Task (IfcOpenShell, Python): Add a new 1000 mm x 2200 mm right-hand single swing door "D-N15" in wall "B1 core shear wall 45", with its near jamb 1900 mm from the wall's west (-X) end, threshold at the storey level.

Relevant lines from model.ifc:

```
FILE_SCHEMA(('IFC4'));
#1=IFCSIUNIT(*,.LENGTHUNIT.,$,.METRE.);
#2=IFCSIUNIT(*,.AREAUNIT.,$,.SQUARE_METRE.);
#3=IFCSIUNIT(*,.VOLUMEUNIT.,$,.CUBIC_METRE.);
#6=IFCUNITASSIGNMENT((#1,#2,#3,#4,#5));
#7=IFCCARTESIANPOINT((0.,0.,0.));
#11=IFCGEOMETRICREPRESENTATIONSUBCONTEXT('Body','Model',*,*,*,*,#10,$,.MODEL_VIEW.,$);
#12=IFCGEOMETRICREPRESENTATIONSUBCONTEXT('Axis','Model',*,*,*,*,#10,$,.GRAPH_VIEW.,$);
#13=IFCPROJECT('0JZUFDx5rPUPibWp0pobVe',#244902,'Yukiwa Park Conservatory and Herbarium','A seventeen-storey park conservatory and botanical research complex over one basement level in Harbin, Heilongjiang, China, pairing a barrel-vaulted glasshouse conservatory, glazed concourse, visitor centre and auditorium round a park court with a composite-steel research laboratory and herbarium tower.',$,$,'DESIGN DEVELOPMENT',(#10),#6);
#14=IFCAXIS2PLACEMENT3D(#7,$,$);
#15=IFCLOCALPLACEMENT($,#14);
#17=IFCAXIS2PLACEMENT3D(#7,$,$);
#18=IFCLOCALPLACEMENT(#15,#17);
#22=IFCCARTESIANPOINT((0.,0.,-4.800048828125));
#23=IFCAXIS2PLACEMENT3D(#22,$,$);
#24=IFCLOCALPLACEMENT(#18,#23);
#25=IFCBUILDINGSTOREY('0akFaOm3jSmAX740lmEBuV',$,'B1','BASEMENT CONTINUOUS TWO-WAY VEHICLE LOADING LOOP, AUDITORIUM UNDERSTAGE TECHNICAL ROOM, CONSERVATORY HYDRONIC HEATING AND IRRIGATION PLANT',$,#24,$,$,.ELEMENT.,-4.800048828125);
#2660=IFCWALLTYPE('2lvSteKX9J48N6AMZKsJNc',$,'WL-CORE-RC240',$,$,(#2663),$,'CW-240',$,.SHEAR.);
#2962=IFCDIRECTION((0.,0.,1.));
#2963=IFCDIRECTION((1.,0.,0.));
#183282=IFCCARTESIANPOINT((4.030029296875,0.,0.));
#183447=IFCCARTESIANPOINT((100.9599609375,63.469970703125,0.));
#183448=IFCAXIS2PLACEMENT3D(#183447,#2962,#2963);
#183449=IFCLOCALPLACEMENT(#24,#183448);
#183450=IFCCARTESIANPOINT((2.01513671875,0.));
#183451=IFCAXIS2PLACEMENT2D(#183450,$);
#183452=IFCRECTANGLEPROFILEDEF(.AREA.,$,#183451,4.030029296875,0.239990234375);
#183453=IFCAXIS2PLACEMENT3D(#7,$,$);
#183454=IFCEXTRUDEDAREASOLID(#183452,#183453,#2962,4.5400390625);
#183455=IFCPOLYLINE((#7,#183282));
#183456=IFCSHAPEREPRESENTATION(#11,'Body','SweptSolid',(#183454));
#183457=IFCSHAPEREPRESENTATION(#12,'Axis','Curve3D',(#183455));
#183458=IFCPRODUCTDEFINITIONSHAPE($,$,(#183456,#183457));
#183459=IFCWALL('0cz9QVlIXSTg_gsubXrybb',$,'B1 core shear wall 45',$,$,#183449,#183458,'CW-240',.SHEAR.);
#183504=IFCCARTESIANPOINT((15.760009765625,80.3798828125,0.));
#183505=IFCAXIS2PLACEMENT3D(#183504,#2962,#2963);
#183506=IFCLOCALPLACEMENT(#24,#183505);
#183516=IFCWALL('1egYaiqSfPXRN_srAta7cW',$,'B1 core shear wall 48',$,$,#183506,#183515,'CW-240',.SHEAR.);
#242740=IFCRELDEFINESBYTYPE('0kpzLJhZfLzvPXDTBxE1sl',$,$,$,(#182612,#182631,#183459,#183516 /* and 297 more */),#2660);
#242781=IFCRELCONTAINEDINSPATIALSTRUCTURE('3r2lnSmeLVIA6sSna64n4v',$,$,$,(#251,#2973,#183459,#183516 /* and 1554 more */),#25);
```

```python
import numpy as np
import ifcopenshell
import ifcopenshell.api.feature
import ifcopenshell.api.geometry
import ifcopenshell.api.root
import ifcopenshell.api.spatial
import ifcopenshell.geom
import ifcopenshell.util.element
import ifcopenshell.util.placement
import ifcopenshell.util.representation
import ifcopenshell.util.shape
import ifcopenshell.util.unit

model = ifcopenshell.open("model.ifc")
unit_scale = ifcopenshell.util.unit.calculate_unit_scale(model)
settings = ifcopenshell.geom.settings()


def volume(element):
    """Net volume in cubic metres, openings subtracted."""
    shape = ifcopenshell.geom.create_shape(settings, element)
    return ifcopenshell.util.shape.get_volume(shape.geometry)


wall = model.by_guid("0cz9QVlIXSTg_gsubXrybb")
storey = ifcopenshell.util.element.get_container(wall, ifc_class="IfcBuildingStorey")
context = ifcopenshell.util.representation.get_context(model, "Model", "Body", "MODEL_VIEW")
before = volume(wall)

width, height, from_end, sill = 1, 2.2, 1.9, 0.0  # metres

# The wall runs along its own X axis, and the end named is its -X end.
wall_shape = ifcopenshell.geom.create_shape(settings, wall)
x, y, z = ifcopenshell.util.shape.get_vertices(wall_shape.geometry).T
start = x.min() + from_end
face, thickness = float(y.min()), float(y.max() - y.min())
wall_matrix = ifcopenshell.util.placement.get_local_placement(wall.ObjectPlacement)
level = ifcopenshell.util.placement.get_local_placement(storey.ObjectPlacement)[2, 3]


def in_wall(x, y):
    """Placement at x, y metres in the wall's axes, at sill height."""
    matrix = wall_matrix.copy()
    matrix[:, 3] = wall_matrix @ np.array([x / unit_scale, y / unit_scale, 0.0, 1.0])
    matrix[2, 3] = level + sill / unit_scale
    return matrix


# Opening: a box that overshoots both wall faces by 50 mm.
opening = ifcopenshell.api.root.create_entity(model, ifc_class="IfcOpeningElement", predefined_type="OPENING")
box = ifcopenshell.api.geometry.add_wall_representation(
    model, context=context, length=width, height=height, thickness=thickness + 0.1
)
ifcopenshell.api.geometry.assign_representation(model, product=opening, representation=box)
ifcopenshell.api.geometry.edit_object_placement(model, product=opening, matrix=in_wall(start, face - 0.05), is_si=False)
ifcopenshell.api.feature.add_feature(model, feature=opening, element=wall)

door = ifcopenshell.api.root.create_entity(model, ifc_class="IfcDoor", name="D-N15", predefined_type="DOOR")
door.OverallWidth, door.OverallHeight = width / unit_scale, height / unit_scale
door.OperationType = "SINGLE_SWING_RIGHT"
body = ifcopenshell.api.geometry.add_door_representation(
    model,
    context=context,
    overall_width=door.OverallWidth,
    overall_height=door.OverallHeight,
    operation_type="SINGLE_SWING_RIGHT",
    lining_properties={"LiningDepth": thickness / unit_scale, "ThresholdDepth": thickness / unit_scale},
)
ifcopenshell.api.geometry.assign_representation(model, product=door, representation=body)
ifcopenshell.api.spatial.assign_container(model, products=[door], relating_structure=storey)
ifcopenshell.api.feature.add_filling(model, opening=opening, element=door)

# The lining spans the wall, so the door starts at the wall face.
ifcopenshell.api.geometry.edit_object_placement(model, product=door, matrix=in_wall(start, face), is_si=False)

after = volume(wall)

print(f"wall volume {before:.3f} -> {after:.3f} m3")

model.write("model_rev.ifc")
```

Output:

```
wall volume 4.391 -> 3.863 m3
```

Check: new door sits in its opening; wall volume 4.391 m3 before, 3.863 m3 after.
